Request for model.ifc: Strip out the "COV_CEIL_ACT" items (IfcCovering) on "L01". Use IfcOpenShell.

First a look at what the model holds.

```python
import ifcopenshell
import ifcopenshell.util.element

model = ifcopenshell.open("model.ifc")
print(model.schema)
storey = next(s for s in model.by_type("IfcBuildingStorey") if s.Name == "L01")
coverings = [e for e in ifcopenshell.util.element.get_decomposition(storey) if e.is_a("IfcCovering")]
seen = {}
for e in coverings:
    element_type = ifcopenshell.util.element.get_type(e)
    name = element_type.Name if element_type not in (None, e) else None
    seen[name] = seen.get(name, 0) + 1
for name, count in sorted(seen.items(), key=str):
    print(count, "x", name)
```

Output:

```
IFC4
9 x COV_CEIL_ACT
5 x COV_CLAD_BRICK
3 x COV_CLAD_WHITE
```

```python
import ifcopenshell
import ifcopenshell.api.root
import ifcopenshell.util.element

model = ifcopenshell.open("model.ifc")

storey = next(s for s in model.by_type("IfcBuildingStorey") if s.Name == "L01")
coverings = [e for e in ifcopenshell.util.element.get_decomposition(storey) if e.is_a("IfcCovering")]
targets = [e for e in coverings if (t := ifcopenshell.util.element.get_type(e)) not in (None, e) and t.Name == "COV_CEIL_ACT"]

for e in targets:
    ifcopenshell.api.root.remove_product(model, product=e)
print(len(targets), "removed")

model.write("model_v2.ifc")
```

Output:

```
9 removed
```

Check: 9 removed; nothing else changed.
